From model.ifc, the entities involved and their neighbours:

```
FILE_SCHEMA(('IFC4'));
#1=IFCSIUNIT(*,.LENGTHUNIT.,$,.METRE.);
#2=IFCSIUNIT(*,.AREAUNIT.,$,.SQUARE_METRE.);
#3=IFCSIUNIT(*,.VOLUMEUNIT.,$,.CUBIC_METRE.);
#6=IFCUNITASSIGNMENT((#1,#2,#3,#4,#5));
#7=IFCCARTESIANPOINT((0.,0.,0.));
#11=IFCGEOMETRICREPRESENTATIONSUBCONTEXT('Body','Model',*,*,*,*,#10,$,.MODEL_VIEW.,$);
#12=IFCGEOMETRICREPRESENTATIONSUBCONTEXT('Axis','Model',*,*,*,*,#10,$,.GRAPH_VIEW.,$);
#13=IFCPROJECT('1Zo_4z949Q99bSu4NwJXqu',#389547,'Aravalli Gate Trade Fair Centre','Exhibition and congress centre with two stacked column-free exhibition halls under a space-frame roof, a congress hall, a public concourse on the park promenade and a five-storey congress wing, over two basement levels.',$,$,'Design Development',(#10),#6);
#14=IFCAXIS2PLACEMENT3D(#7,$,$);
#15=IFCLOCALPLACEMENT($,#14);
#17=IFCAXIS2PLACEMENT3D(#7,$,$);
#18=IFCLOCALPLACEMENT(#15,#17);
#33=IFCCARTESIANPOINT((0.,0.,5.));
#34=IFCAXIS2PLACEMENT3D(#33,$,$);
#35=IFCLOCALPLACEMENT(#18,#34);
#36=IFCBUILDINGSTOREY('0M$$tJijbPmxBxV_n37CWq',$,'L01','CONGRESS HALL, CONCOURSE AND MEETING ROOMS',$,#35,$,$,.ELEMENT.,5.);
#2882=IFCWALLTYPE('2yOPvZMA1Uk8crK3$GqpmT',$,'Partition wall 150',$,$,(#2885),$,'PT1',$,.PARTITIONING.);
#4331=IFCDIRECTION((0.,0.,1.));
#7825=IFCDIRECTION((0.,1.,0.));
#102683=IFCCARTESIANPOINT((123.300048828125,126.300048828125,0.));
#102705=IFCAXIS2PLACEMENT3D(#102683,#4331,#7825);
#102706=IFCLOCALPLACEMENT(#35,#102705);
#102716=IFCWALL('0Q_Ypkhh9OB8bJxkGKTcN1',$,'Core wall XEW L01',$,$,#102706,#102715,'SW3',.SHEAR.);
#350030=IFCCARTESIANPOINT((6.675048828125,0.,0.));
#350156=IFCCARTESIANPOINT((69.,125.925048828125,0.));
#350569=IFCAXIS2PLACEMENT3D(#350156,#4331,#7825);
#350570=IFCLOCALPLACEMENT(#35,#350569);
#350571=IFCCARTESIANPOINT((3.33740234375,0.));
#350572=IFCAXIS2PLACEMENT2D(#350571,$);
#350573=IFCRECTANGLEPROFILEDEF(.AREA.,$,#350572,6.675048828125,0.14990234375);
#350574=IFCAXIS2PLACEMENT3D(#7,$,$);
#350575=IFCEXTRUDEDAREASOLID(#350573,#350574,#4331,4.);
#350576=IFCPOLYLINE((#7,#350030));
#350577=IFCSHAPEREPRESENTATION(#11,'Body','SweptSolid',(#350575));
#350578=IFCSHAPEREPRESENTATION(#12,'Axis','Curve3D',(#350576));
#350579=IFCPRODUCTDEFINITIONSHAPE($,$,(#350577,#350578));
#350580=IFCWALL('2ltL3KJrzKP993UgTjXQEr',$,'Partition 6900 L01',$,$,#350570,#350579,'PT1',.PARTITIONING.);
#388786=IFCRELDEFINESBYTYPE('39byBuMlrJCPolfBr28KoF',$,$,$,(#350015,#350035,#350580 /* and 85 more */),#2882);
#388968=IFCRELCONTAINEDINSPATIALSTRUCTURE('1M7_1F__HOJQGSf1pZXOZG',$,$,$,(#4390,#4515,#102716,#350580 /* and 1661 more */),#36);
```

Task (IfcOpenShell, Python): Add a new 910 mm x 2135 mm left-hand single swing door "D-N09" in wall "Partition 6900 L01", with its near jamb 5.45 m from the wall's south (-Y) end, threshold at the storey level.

```python
import numpy as np
import ifcopenshell
import ifcopenshell.api.feature
import ifcopenshell.api.geometry
import ifcopenshell.api.root
import ifcopenshell.api.spatial
import ifcopenshell.geom
import ifcopenshell.util.element
import ifcopenshell.util.placement
import ifcopenshell.util.representation
import ifcopenshell.util.shape
import ifcopenshell.util.unit

model = ifcopenshell.open("model.ifc")
unit_scale = ifcopenshell.util.unit.calculate_unit_scale(model)
settings = ifcopenshell.geom.settings()


def volume(element):
    """Net volume in cubic metres, openings subtracted."""
    shape = ifcopenshell.geom.create_shape(settings, element)
    return ifcopenshell.util.shape.get_volume(shape.geometry)


wall = model.by_id(350580)
storey = ifcopenshell.util.element.get_container(wall, ifc_class="IfcBuildingStorey")
context = ifcopenshell.util.representation.get_context(model, "Model", "Body", "MODEL_VIEW")
before = volume(wall)

width, height, from_end, sill = 0.91, 2.135, 5.45, 0.0  # metres

# The wall runs along its own X axis, and the end named is its -X end.
wall_shape = ifcopenshell.geom.create_shape(settings, wall)
x, y, z = ifcopenshell.util.shape.get_vertices(wall_shape.geometry).T
start = x.min() + from_end
face, thickness = float(y.min()), float(y.max() - y.min())
wall_matrix = ifcopenshell.util.placement.get_local_placement(wall.ObjectPlacement)
level = ifcopenshell.util.placement.get_local_placement(storey.ObjectPlacement)[2, 3]


def in_wall(x, y):
    """Placement at x, y metres in the wall's axes, at sill height."""
    matrix = wall_matrix.copy()
    matrix[:, 3] = wall_matrix @ np.array([x / unit_scale, y / unit_scale, 0.0, 1.0])
    matrix[2, 3] = level + sill / unit_scale
    return matrix


# Opening: a box that overshoots both wall faces by 50 mm.
opening = ifcopenshell.api.root.create_entity(model, ifc_class="IfcOpeningElement", predefined_type="OPENING")
box = ifcopenshell.api.geometry.add_wall_representation(
    model, context=context, length=width, height=height, thickness=thickness + 0.1
)
ifcopenshell.api.geometry.assign_representation(model, product=opening, representation=box)
ifcopenshell.api.geometry.edit_object_placement(model, product=opening, matrix=in_wall(start, face - 0.05), is_si=False)
ifcopenshell.api.feature.add_feature(model, feature=opening, element=wall)

door = ifcopenshell.api.root.create_entity(model, ifc_class="IfcDoor", name="D-N09", predefined_type="DOOR")
door.OverallWidth, door.OverallHeight = width / unit_scale, height / unit_scale
door.OperationType = "SINGLE_SWING_LEFT"
body = ifcopenshell.api.geometry.add_door_representation(
    model,
    context=context,
    overall_width=door.OverallWidth,
    overall_height=door.OverallHeight,
    operation_type="SINGLE_SWING_LEFT",
    lining_properties={"LiningDepth": thickness / unit_scale, "ThresholdDepth": thickness / unit_scale},
)
ifcopenshell.api.geometry.assign_representation(model, product=door, representation=body)
ifcopenshell.api.spatial.assign_container(model, products=[door], relating_structure=storey)
ifcopenshell.api.feature.add_filling(model, opening=opening, element=door)

# The lining spans the wall, so the door starts at the wall face.
ifcopenshell.api.geometry.edit_object_placement(model, product=door, matrix=in_wall(start, face), is_si=False)

after = volume(wall)

print(f"wall volume {before:.3f} -> {after:.3f} m3")

model.write("model-out.ifc")
```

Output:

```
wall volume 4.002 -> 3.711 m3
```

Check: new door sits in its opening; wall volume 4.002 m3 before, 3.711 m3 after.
